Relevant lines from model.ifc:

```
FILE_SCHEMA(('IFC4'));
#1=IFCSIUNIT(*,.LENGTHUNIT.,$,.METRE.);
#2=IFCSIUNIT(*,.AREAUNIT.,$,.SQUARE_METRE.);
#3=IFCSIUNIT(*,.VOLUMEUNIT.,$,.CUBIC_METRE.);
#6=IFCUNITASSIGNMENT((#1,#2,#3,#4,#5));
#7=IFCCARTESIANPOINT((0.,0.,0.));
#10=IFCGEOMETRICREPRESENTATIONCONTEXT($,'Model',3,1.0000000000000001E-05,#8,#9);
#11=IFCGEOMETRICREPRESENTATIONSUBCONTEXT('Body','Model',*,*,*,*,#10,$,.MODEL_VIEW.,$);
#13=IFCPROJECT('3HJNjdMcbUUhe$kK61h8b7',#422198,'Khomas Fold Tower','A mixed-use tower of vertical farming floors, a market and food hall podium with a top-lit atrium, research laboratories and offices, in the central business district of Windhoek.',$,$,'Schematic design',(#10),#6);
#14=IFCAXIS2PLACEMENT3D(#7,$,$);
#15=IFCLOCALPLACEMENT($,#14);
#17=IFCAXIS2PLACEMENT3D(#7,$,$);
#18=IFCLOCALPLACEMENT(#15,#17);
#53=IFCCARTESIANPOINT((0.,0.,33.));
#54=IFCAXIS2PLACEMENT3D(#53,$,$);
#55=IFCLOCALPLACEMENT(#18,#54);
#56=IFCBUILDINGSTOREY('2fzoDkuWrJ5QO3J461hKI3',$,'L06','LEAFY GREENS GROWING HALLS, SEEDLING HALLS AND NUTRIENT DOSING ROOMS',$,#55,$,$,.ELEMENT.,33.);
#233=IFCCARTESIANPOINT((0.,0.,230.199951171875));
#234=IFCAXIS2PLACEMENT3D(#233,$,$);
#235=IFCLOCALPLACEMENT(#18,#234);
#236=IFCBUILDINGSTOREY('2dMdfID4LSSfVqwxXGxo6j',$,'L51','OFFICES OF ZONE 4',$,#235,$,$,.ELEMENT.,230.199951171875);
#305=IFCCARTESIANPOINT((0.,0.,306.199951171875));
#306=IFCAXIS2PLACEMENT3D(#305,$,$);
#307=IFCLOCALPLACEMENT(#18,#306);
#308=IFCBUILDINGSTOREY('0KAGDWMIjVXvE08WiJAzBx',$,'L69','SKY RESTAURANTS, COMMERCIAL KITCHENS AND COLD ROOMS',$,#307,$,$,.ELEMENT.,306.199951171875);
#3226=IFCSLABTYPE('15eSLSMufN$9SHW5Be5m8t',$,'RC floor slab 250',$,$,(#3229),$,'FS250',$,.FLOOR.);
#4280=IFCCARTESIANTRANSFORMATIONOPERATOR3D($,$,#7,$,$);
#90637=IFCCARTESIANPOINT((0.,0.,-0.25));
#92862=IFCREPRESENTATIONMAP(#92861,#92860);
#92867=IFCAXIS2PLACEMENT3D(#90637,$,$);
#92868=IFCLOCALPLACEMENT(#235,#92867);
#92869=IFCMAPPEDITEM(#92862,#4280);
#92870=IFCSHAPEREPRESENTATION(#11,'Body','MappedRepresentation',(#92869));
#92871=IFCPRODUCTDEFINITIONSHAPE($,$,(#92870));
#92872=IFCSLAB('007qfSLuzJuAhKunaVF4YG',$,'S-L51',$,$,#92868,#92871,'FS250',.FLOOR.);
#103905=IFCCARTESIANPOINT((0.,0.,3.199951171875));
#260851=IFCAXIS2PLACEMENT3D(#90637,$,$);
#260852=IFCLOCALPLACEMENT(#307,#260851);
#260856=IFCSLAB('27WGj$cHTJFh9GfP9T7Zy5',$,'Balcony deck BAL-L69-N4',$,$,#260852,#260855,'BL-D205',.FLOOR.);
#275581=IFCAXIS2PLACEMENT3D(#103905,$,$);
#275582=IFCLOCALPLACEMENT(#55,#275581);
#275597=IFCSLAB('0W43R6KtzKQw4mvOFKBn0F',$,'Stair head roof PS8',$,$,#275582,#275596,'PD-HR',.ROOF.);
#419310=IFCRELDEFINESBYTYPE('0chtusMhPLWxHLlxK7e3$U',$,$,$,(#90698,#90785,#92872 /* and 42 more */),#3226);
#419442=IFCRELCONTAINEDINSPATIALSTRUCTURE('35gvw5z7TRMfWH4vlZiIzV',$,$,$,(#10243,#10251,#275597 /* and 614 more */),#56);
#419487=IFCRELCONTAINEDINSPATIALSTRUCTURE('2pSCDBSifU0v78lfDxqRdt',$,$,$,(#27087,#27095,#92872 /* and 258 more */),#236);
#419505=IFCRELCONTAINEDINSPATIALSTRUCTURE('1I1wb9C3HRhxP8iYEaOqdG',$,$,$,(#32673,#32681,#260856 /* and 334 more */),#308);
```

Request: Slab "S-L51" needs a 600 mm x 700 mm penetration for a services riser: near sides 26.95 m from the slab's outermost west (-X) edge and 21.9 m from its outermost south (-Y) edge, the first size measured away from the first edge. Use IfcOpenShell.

```python
import numpy as np
import ifcopenshell
import ifcopenshell.api.feature
import ifcopenshell.api.geometry
import ifcopenshell.api.root
import ifcopenshell.geom
import ifcopenshell.util.placement
import ifcopenshell.util.representation
import ifcopenshell.util.shape
import ifcopenshell.util.unit

model = ifcopenshell.open("model.ifc")
unit_scale = ifcopenshell.util.unit.calculate_unit_scale(model)
settings = ifcopenshell.geom.settings()


def volume(element):
    """Net volume in cubic metres, openings subtracted."""
    shape = ifcopenshell.geom.create_shape(settings, element)
    return ifcopenshell.util.shape.get_volume(shape.geometry)


slab = model.by_guid("007qfSLuzJuAhKunaVF4YG")
before = volume(slab)

# Extent in the slab's own axes, in metres. The edges named are its -X and -Y sides.
slab_shape = ifcopenshell.geom.create_shape(settings, slab)
vertices = ifcopenshell.util.shape.get_vertices(slab_shape.geometry)
x_min, y_min, bottom = vertices.min(axis=0)
top = vertices[:, 2].max()

opening = ifcopenshell.api.root.create_entity(model, ifc_class="IfcOpeningElement", name="Services riser opening", predefined_type="OPENING")
context = ifcopenshell.util.representation.get_context(model, "Model", "Body", "MODEL_VIEW")
width, depth = 0.6, 0.7
outline = [(0.0, 0.0), (width, 0.0), (width, depth), (0.0, depth), (0.0, 0.0)]
# Overshoot both faces by 50 mm so the cut is clean.
shape = ifcopenshell.api.geometry.add_slab_representation(
    model, context=context, depth=top - bottom + 0.1, polyline=outline
)
ifcopenshell.api.geometry.assign_representation(model, product=opening, representation=shape)

matrix = ifcopenshell.util.placement.get_local_placement(slab.ObjectPlacement)
matrix[:, 3] = matrix @ np.append(np.array([x_min + 26.95, y_min + 21.9, bottom - 0.05]) / unit_scale, 1.0)
ifcopenshell.api.geometry.edit_object_placement(model, product=opening, matrix=matrix, is_si=False)
ifcopenshell.api.feature.add_feature(model, feature=opening, element=slab)

after = volume(slab)

print(f"slab volume {before:.3f} -> {after:.3f} m3")

model.write("model_rev.ifc")
```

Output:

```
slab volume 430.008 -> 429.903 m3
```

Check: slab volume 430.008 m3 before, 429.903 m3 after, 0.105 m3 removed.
